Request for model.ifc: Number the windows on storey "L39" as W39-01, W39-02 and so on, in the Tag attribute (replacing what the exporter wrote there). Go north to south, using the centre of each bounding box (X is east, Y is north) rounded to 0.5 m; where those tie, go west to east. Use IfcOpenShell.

First a look at what the model holds.

```python
import ifcopenshell
import ifcopenshell.util.element
import ifcopenshell.util.placement

model = ifcopenshell.open("model.ifc")
print(model.schema)
storey = next(s for s in model.by_type("IfcBuildingStorey") if s.Name == "L39")
windows = [e for e in ifcopenshell.util.element.get_decomposition(storey) if e.is_a("IfcWindow")]
for e in sorted(windows, key=lambda e: e.id()):
    origin = ifcopenshell.util.placement.get_local_placement(e.ObjectPlacement)[:3, 3]
    print(e.id(), e.Tag, e.Name, origin.round(2) + 0.0, sep=" | ")
```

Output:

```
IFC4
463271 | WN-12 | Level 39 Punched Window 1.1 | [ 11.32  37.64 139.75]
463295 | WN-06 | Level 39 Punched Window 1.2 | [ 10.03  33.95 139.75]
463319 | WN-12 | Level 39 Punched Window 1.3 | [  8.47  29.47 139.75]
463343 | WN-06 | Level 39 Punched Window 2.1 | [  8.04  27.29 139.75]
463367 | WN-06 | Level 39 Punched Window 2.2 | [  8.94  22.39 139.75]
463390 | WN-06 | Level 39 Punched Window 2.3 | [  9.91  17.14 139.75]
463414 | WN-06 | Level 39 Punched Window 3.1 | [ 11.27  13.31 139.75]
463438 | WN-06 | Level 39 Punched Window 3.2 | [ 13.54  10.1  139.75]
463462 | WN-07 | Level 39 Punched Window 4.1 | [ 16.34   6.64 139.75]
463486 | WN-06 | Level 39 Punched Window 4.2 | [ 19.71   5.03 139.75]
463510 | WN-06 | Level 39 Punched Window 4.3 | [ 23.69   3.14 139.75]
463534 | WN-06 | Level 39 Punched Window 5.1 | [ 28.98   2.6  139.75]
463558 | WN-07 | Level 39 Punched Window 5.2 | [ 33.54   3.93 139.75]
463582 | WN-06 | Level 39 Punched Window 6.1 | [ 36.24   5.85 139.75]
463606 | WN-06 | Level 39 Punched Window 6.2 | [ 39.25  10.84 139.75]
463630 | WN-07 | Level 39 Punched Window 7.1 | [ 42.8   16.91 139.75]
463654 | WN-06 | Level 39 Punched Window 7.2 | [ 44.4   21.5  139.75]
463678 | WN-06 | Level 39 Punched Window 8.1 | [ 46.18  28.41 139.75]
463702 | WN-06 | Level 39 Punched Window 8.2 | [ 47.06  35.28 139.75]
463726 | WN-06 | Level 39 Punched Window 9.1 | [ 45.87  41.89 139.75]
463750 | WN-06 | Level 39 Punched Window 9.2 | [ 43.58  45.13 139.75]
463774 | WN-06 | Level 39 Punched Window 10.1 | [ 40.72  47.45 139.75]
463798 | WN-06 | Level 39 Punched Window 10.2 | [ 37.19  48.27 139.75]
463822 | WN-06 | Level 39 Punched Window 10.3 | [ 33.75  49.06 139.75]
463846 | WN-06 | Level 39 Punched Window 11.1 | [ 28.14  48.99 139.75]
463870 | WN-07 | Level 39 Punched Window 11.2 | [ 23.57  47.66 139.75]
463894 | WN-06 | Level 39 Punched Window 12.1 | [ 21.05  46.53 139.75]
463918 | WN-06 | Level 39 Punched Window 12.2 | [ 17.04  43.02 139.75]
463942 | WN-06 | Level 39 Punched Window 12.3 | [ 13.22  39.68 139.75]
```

```python
import ifcopenshell
import ifcopenshell.geom
import ifcopenshell.util.element
import ifcopenshell.util.shape

model = ifcopenshell.open("model.ifc")
settings = ifcopenshell.geom.settings()
settings.set("use-world-coords", True)


def centre(element):
    shape = ifcopenshell.geom.create_shape(settings, element)
    return ifcopenshell.util.shape.get_bbox_centroid(shape.geometry)


storey = next(s for s in model.by_type("IfcBuildingStorey") if s.Name == "L39")
windows = [e for e in ifcopenshell.util.element.get_decomposition(storey) if e.is_a("IfcWindow")]

# Insertion points can sit at a corner or the storey origin, so sort by the geometry (in metres).
centres = {e: centre(e) for e in windows}
windows.sort(key=lambda e: (-round(centres[e][1] / 0.5), centres[e][0]))

for i, e in enumerate(windows, start=1):
    number = f"W39-{i:02d}"
    e.Tag = number
    print(e.id(), number)

model.write("model_updated.ifc")
```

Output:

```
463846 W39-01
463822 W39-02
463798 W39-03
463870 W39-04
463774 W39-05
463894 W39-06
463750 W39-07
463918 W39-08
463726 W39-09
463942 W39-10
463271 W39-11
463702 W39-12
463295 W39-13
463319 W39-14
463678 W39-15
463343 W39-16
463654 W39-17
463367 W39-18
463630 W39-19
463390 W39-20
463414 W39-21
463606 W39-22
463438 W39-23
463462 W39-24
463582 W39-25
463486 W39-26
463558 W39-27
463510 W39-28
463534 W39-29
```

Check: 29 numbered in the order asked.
